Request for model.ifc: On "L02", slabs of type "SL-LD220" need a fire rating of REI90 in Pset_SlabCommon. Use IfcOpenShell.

First a look at what the model holds.

```python
import ifcopenshell
import ifcopenshell.util.element

model = ifcopenshell.open("model.ifc")
print(model.schema)
storey = next(s for s in model.by_type("IfcBuildingStorey") if s.Name == "L02")
slabs = [e for e in ifcopenshell.util.element.get_decomposition(storey) if e.is_a("IfcSlab")]
seen = {}
for e in slabs:
    element_type = ifcopenshell.util.element.get_type(e)
    key = (element_type.Name if element_type != e and element_type else None, ifcopenshell.util.element.get_pset(e, "Pset_SlabCommon", "FireRating"))
    seen[key] = seen.get(key, 0) + 1
for (name, value), count in sorted(seen.items(), key=str):
    print(count, "x", name, "|", value)
```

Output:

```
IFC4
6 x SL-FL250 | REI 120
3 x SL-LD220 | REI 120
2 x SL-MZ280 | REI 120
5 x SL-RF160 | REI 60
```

```python
import ifcopenshell
import ifcopenshell.api.pset
import ifcopenshell.util.element

model = ifcopenshell.open("model.ifc")

storey = next(s for s in model.by_type("IfcBuildingStorey") if s.Name == "L02")
slabs = [e for e in ifcopenshell.util.element.get_decomposition(storey) if e.is_a("IfcSlab")]

count = 0
for e in slabs:
    element_type = ifcopenshell.util.element.get_type(e)
    if element_type in (None, e) or element_type.Name != "SL-LD220":
        continue
    # add_pset returns the element's existing set when there is one.
    pset = ifcopenshell.api.pset.add_pset(model, product=e, name="Pset_SlabCommon")
    ifcopenshell.api.pset.edit_pset(model, pset=pset, properties={"FireRating": "REI90"})
    count += 1

print(count, "slabs updated")

model.write("model-out.ifc")
```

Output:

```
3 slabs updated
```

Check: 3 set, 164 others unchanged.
